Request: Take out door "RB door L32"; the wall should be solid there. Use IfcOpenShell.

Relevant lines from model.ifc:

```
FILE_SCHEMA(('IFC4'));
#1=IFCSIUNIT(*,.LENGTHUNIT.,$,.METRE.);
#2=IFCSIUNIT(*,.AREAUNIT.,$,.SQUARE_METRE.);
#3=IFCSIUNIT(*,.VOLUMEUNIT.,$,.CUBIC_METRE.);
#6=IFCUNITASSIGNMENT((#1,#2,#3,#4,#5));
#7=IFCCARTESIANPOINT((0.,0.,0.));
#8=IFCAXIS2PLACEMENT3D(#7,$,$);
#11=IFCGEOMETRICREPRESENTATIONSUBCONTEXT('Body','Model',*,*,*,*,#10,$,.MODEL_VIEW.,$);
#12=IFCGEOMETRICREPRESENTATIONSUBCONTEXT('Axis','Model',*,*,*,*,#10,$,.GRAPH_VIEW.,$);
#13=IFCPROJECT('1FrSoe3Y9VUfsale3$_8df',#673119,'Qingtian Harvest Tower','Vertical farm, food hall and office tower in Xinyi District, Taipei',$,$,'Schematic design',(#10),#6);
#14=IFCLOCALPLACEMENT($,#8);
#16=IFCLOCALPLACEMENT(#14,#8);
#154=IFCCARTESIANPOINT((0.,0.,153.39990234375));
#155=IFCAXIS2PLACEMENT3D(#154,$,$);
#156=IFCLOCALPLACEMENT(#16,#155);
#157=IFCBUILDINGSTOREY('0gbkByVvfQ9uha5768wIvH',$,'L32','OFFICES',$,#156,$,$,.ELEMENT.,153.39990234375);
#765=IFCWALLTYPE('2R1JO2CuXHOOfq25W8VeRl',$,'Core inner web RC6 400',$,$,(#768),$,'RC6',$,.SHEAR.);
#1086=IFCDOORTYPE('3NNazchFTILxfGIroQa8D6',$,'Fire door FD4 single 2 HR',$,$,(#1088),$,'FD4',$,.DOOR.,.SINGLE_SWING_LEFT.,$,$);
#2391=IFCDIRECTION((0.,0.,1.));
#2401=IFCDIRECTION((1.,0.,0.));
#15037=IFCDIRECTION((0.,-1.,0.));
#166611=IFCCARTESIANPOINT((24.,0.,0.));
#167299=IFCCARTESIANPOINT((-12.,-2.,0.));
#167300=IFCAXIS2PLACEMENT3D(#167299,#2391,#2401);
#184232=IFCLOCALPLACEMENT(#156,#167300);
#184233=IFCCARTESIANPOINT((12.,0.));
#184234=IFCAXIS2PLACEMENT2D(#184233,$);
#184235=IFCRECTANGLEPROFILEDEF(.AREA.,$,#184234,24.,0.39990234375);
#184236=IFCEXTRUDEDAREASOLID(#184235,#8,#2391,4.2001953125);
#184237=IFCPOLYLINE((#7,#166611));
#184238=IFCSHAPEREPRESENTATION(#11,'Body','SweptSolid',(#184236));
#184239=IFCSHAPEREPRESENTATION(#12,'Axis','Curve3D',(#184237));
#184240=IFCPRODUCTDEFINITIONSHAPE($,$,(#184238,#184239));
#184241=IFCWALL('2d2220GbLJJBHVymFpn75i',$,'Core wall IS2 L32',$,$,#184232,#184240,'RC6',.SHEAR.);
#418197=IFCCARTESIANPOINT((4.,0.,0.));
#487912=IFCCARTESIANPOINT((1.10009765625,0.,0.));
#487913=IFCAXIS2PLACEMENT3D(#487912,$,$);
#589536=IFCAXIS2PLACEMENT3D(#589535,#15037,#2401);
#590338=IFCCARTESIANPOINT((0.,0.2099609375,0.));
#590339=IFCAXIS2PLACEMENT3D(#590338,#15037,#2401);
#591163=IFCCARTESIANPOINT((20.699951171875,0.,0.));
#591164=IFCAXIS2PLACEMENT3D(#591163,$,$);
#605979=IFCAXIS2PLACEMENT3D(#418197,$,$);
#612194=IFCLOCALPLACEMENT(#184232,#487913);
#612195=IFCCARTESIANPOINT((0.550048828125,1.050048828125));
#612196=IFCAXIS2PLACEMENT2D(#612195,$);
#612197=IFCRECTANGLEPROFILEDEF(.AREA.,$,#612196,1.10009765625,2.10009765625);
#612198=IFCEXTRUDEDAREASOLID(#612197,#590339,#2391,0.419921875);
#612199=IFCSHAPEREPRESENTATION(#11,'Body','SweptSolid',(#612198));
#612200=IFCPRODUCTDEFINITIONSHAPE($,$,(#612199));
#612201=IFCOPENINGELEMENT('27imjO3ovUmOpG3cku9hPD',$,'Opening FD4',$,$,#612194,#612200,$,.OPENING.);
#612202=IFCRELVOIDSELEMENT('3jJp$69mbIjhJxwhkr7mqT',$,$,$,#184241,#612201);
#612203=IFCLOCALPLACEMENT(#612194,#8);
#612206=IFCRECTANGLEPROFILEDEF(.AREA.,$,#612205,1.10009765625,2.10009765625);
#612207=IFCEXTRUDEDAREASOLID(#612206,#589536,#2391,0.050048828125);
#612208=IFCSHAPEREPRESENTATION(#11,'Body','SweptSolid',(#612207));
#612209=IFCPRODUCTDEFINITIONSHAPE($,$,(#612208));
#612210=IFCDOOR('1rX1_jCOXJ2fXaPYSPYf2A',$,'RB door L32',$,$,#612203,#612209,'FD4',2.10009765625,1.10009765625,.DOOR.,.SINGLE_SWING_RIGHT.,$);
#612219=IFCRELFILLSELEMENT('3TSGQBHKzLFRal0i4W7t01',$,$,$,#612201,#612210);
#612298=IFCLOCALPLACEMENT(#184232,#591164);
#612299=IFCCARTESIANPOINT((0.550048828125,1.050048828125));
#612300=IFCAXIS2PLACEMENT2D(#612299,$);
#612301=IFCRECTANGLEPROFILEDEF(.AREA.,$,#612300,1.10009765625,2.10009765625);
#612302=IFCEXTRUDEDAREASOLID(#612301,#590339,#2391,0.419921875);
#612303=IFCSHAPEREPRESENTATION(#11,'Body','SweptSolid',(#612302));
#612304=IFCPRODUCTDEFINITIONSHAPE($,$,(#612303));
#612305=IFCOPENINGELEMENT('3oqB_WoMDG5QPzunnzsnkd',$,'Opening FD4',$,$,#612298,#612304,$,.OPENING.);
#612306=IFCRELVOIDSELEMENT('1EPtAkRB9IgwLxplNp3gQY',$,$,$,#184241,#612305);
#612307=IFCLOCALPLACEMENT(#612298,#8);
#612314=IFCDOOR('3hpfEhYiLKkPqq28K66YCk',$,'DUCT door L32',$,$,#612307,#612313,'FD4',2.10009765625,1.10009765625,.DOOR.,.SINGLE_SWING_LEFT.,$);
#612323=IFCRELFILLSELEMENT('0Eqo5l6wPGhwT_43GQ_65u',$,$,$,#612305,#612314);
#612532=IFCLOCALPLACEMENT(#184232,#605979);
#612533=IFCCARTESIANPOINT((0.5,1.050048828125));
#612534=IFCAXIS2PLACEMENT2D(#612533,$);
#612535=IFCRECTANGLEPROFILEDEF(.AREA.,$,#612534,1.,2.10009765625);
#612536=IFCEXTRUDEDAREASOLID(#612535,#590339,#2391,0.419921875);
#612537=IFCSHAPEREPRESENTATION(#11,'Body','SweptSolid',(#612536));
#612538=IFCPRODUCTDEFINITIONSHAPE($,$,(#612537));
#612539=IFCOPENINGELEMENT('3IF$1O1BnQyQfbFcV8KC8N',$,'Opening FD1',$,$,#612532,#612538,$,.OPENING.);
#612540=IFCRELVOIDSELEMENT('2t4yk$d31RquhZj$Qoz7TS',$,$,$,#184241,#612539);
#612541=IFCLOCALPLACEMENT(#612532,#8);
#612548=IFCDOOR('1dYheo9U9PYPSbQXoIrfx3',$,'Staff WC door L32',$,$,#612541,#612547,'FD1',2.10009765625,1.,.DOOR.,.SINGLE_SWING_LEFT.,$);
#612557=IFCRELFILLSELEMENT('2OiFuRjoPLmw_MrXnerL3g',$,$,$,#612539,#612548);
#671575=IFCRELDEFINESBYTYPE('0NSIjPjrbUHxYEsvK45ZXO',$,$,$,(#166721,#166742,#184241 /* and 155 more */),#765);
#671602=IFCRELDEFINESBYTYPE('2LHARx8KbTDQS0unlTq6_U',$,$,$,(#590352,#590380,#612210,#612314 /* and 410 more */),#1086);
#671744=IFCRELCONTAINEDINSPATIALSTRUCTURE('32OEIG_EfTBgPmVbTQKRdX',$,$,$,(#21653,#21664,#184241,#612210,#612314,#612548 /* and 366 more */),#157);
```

```python
import ifcopenshell
import ifcopenshell.api.feature
import ifcopenshell.api.root
import ifcopenshell.geom
import ifcopenshell.util.shape

model = ifcopenshell.open("model.ifc")
settings = ifcopenshell.geom.settings()


def volume(element):
    """Net volume in cubic metres, openings subtracted."""
    shape = ifcopenshell.geom.create_shape(settings, element)
    return ifcopenshell.util.shape.get_volume(shape.geometry)


door = model.by_id(612210)
opening = door.FillsVoids[0].RelatingOpeningElement
wall = opening.VoidsElements[0].RelatingBuildingElement
before = volume(wall)

ifcopenshell.api.root.remove_product(model, product=door)
ifcopenshell.api.feature.remove_feature(model, feature=opening)

after = volume(wall)

print(f"wall volume {before:.3f} -> {after:.3f} m3")

model.write("model_updated.ifc")
```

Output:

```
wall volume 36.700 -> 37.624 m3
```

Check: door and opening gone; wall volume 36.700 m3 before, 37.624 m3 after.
